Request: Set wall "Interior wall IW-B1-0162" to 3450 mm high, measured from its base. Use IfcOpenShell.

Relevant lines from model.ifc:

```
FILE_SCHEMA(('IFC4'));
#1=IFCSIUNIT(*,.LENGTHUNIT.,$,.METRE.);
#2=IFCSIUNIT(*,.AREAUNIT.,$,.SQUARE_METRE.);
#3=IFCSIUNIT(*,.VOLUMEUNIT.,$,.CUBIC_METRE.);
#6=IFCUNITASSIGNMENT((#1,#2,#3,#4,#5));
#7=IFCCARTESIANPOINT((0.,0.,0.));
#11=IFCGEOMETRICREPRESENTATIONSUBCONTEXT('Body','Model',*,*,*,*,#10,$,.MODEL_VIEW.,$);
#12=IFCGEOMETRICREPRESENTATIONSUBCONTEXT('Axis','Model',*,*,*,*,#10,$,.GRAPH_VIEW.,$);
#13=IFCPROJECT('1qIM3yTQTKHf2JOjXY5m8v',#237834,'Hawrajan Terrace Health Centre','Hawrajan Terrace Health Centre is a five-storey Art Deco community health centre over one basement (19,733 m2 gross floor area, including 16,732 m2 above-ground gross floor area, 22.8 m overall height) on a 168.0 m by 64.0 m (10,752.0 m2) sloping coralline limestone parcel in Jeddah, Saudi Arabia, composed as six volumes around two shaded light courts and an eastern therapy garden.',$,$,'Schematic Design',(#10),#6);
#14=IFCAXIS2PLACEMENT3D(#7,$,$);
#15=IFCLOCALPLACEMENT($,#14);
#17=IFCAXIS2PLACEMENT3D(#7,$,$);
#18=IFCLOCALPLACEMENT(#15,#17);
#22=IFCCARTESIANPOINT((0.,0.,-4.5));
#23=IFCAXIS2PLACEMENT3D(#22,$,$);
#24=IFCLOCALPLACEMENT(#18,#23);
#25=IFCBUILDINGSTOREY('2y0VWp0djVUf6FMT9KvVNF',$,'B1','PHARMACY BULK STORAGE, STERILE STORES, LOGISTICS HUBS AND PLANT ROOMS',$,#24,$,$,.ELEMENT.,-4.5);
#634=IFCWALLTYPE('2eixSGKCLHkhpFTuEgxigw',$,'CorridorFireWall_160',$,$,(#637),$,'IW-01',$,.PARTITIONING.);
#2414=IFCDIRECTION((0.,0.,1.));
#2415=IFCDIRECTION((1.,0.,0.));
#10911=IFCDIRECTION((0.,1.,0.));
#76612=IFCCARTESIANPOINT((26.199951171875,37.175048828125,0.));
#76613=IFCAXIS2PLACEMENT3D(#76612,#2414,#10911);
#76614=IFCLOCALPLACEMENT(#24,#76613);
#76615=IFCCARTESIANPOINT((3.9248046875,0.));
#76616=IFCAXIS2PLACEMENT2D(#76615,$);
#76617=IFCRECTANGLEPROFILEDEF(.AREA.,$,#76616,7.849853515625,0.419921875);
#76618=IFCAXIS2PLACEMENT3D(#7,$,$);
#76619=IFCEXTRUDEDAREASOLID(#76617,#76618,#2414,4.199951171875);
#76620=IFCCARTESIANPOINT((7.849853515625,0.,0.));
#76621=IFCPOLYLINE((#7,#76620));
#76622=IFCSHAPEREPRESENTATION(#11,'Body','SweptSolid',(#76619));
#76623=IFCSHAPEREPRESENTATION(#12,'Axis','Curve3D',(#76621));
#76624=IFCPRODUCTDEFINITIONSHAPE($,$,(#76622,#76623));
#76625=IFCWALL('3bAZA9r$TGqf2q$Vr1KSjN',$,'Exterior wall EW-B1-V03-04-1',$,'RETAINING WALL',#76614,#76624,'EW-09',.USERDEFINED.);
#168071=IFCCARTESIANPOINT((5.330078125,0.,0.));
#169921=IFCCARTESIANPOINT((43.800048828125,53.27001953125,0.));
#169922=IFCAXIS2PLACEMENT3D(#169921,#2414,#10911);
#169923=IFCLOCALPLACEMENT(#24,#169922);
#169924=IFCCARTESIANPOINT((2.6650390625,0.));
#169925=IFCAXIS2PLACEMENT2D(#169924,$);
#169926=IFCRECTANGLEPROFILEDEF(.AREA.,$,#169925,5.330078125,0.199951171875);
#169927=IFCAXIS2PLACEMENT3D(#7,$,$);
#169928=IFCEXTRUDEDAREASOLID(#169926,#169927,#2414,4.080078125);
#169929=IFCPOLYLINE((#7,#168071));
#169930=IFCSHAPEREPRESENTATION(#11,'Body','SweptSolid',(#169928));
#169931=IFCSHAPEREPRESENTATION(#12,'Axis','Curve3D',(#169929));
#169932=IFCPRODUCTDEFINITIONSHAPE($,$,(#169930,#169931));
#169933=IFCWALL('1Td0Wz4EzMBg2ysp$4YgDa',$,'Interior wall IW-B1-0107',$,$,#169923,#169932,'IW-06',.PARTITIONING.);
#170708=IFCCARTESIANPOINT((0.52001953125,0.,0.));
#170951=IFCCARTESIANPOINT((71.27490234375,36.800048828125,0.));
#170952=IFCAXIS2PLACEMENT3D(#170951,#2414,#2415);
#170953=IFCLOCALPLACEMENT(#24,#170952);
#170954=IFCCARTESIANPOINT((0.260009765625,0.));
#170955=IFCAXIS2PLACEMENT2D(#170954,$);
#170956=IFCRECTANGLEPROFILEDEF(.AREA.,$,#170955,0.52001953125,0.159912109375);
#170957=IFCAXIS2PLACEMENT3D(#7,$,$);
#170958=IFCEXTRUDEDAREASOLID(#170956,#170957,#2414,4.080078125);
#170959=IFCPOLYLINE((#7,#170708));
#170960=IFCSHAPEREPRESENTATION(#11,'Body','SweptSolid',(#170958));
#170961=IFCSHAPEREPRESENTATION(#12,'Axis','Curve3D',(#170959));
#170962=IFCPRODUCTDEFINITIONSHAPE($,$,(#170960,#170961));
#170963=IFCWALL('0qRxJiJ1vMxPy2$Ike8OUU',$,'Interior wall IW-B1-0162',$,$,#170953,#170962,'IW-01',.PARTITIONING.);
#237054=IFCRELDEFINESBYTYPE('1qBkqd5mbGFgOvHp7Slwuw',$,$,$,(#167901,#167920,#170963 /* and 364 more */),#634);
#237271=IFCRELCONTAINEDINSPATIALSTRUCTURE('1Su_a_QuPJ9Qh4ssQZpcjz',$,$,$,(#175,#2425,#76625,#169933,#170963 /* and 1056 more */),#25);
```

```python
import ifcopenshell
import ifcopenshell.geom
import ifcopenshell.util.representation
import ifcopenshell.util.shape
import ifcopenshell.util.unit

model = ifcopenshell.open("model.ifc")
unit_scale = ifcopenshell.util.unit.calculate_unit_scale(model)
settings = ifcopenshell.geom.settings()


def volume(element):
    """Net volume in cubic metres, openings subtracted."""
    shape = ifcopenshell.geom.create_shape(settings, element)
    return ifcopenshell.util.shape.get_volume(shape.geometry)


wall = model.by_guid("0qRxJiJ1vMxPy2$Ike8OUU")
before = volume(wall)

body = ifcopenshell.util.representation.get_representation(wall, "Model", "Body")
solid = body.Items[0]
old_height = solid.Depth
solid.Depth = 3.45 / unit_scale
after = volume(wall)

print(f"height {old_height:g} -> {solid.Depth:g}, volume {before:.3f} -> {after:.3f} m3")

model.write("model-out.ifc")
```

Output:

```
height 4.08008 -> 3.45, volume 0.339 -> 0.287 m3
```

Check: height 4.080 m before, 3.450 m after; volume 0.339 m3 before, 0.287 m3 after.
